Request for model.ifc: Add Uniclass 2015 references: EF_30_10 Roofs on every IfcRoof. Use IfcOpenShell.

First a look at what the model holds.

```python
import ifcopenshell

model = ifcopenshell.open("model.ifc")
print(model.schema)
print("classifications:", [c.Name for c in model.by_type("IfcClassification")])
for ifc_class in ("IfcDoor", "IfcRoof", "IfcStair", "IfcWall", "IfcWindow"):
    print(ifc_class, len(model.by_type(ifc_class)))
```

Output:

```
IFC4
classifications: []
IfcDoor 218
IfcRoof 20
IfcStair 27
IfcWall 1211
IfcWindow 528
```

```python
import ifcopenshell
import ifcopenshell.api.classification

model = ifcopenshell.open("model.ifc")

system = ifcopenshell.api.classification.add_classification(model, classification="Uniclass 2015")

codes = {
    "IfcRoof": ("EF_30_10", "Roofs"),
}
for ifc_class, (code, name) in codes.items():
    products = model.by_type(ifc_class)
    ifcopenshell.api.classification.add_reference(
        model, products=products, classification=system, identification=code, name=name
    )
    print(code, len(products))

model.write("model_edited.ifc")
```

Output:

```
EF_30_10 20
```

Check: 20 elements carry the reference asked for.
